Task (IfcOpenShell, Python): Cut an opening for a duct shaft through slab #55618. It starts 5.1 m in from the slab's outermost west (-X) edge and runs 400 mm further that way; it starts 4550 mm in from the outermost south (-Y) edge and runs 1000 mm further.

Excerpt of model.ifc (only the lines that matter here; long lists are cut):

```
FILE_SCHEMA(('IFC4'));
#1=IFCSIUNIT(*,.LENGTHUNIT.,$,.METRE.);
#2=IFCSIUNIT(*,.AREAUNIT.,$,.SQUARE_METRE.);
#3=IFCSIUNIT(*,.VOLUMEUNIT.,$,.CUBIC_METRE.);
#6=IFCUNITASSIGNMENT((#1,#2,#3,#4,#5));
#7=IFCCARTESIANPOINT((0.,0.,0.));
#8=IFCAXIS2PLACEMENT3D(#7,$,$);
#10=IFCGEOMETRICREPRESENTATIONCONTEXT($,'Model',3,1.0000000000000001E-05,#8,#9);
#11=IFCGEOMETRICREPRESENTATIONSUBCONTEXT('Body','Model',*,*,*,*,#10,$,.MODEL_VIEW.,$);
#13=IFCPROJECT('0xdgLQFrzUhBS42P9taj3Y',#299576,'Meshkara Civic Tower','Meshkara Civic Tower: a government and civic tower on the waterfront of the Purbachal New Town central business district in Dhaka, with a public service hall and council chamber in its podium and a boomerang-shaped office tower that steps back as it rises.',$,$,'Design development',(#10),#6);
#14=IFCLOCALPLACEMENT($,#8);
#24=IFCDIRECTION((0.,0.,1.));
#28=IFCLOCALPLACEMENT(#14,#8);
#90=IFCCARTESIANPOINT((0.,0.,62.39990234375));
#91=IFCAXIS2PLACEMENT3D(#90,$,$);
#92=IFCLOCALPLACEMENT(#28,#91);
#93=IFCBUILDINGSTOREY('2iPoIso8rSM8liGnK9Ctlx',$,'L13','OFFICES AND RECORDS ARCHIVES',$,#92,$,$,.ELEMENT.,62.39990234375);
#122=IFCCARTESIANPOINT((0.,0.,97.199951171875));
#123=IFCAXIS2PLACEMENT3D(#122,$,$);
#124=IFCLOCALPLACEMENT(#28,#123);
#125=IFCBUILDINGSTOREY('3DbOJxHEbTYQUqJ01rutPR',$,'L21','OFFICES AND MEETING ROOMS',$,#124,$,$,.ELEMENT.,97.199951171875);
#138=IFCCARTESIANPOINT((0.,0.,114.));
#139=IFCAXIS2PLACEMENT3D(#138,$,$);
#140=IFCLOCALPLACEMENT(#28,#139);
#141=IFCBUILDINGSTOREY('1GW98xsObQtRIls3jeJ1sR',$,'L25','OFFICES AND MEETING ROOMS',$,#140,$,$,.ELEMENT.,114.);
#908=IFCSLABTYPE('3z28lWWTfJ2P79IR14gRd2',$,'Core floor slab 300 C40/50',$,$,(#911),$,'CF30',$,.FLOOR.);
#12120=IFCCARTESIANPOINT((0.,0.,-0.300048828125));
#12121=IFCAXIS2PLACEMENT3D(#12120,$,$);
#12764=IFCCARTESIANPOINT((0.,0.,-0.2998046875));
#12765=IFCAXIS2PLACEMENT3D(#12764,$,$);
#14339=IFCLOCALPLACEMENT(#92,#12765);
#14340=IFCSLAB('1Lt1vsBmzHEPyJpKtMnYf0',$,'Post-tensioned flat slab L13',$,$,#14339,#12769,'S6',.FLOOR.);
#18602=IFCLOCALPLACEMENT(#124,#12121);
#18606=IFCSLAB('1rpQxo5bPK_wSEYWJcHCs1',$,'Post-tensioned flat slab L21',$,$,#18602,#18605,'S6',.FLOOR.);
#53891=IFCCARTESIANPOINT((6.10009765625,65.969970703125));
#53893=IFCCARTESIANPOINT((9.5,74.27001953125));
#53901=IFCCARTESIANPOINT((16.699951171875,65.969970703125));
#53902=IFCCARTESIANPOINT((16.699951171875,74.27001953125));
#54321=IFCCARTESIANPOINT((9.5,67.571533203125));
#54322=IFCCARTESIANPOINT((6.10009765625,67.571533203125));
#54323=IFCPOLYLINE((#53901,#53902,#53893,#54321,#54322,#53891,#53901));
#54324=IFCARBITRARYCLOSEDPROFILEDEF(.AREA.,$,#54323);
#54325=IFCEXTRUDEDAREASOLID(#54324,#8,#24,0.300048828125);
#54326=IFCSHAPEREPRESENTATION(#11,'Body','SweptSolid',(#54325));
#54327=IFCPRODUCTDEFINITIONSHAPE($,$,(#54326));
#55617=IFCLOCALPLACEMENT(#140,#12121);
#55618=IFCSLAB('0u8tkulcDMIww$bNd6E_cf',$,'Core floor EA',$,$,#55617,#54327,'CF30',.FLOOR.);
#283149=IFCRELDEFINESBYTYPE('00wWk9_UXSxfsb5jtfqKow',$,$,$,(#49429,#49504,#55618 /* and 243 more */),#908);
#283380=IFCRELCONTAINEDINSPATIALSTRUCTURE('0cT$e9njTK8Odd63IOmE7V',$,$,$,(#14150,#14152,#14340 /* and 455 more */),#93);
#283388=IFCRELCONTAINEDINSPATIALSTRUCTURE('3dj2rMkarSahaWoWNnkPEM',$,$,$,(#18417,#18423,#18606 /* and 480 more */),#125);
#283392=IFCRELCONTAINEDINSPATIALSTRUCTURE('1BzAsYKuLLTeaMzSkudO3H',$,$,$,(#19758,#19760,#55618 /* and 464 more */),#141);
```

```python
import numpy as np
import ifcopenshell
import ifcopenshell.api.feature
import ifcopenshell.api.geometry
import ifcopenshell.api.root
import ifcopenshell.geom
import ifcopenshell.util.placement
import ifcopenshell.util.representation
import ifcopenshell.util.shape
import ifcopenshell.util.unit

model = ifcopenshell.open("model.ifc")
unit_scale = ifcopenshell.util.unit.calculate_unit_scale(model)
settings = ifcopenshell.geom.settings()


def volume(element):
    """Net volume in cubic metres, openings subtracted."""
    shape = ifcopenshell.geom.create_shape(settings, element)
    return ifcopenshell.util.shape.get_volume(shape.geometry)


slab = model.by_guid("0u8tkulcDMIww$bNd6E_cf")
before = volume(slab)

# Extent in the slab's own axes, in metres. The edges named are its -X and -Y sides.
slab_shape = ifcopenshell.geom.create_shape(settings, slab)
vertices = ifcopenshell.util.shape.get_vertices(slab_shape.geometry)
x_min, y_min, bottom = vertices.min(axis=0)
top = vertices[:, 2].max()

opening = ifcopenshell.api.root.create_entity(model, ifc_class="IfcOpeningElement", name="Duct shaft opening", predefined_type="OPENING")
context = ifcopenshell.util.representation.get_context(model, "Model", "Body", "MODEL_VIEW")
width, depth = 0.4, 1
outline = [(0.0, 0.0), (width, 0.0), (width, depth), (0.0, depth), (0.0, 0.0)]
# Overshoot both faces by 50 mm so the cut is clean.
shape = ifcopenshell.api.geometry.add_slab_representation(
    model, context=context, depth=top - bottom + 0.1, polyline=outline
)
ifcopenshell.api.geometry.assign_representation(model, product=opening, representation=shape)

matrix = ifcopenshell.util.placement.get_local_placement(slab.ObjectPlacement)
matrix[:, 3] = matrix @ np.append(np.array([x_min + 5.1, y_min + 4.55, bottom - 0.05]) / unit_scale, 1.0)
ifcopenshell.api.geometry.edit_object_placement(model, product=opening, matrix=matrix, is_si=False)
ifcopenshell.api.feature.add_feature(model, feature=opening, element=slab)

after = volume(slab)

print(f"slab volume {before:.3f} -> {after:.3f} m3")

model.write("model-out.ifc")
```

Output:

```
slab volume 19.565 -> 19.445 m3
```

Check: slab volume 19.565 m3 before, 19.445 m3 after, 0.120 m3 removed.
